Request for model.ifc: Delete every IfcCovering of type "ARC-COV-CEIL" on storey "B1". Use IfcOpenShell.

First a look at what the model holds.

```python
import ifcopenshell
import ifcopenshell.util.element

model = ifcopenshell.open("model.ifc")
print(model.schema)
storey = next(s for s in model.by_type("IfcBuildingStorey") if s.Name == "B1")
coverings = [e for e in ifcopenshell.util.element.get_decomposition(storey) if e.is_a("IfcCovering")]
seen = {}
for e in coverings:
    element_type = ifcopenshell.util.element.get_type(e)
    name = element_type.Name if element_type not in (None, e) else None
    seen[name] = seen.get(name, 0) + 1
for name, count in sorted(seen.items(), key=str):
    print(count, "x", name)
```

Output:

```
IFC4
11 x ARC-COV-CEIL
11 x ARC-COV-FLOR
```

```python
import ifcopenshell
import ifcopenshell.api.root
import ifcopenshell.util.element

model = ifcopenshell.open("model.ifc")

storey = next(s for s in model.by_type("IfcBuildingStorey") if s.Name == "B1")
coverings = [e for e in ifcopenshell.util.element.get_decomposition(storey) if e.is_a("IfcCovering")]
targets = [e for e in coverings if (t := ifcopenshell.util.element.get_type(e)) not in (None, e) and t.Name == "ARC-COV-CEIL"]

for e in targets:
    ifcopenshell.api.root.remove_product(model, product=e)
print(len(targets), "removed")

model.write("model_edited.ifc")
```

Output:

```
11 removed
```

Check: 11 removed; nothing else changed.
